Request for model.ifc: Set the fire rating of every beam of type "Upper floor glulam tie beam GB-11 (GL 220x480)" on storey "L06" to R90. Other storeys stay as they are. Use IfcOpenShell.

First a look at what the model holds.

```python
import ifcopenshell
import ifcopenshell.util.element

model = ifcopenshell.open("model.ifc")
print(model.schema)
storey = next(s for s in model.by_type("IfcBuildingStorey") if s.Name == "L06")
beams = [e for e in ifcopenshell.util.element.get_decomposition(storey) if e.is_a("IfcBeam")]
seen = {}
for e in beams:
    element_type = ifcopenshell.util.element.get_type(e)
    key = (element_type.Name if element_type != e and element_type else None, ifcopenshell.util.element.get_pset(e, "Pset_BeamCommon", "FireRating"))
    seen[key] = seen.get(key, 0) + 1
for (name, value), count in sorted(seen.items(), key=str):
    print(count, "x", name, "|", value)
```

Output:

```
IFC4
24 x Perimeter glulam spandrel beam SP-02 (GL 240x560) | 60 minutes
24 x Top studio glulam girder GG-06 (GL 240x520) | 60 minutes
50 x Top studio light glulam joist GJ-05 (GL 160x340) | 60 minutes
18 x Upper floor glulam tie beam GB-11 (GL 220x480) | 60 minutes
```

```python
import ifcopenshell
import ifcopenshell.api.pset
import ifcopenshell.util.element

model = ifcopenshell.open("model.ifc")

storey = next(s for s in model.by_type("IfcBuildingStorey") if s.Name == "L06")
beams = [e for e in ifcopenshell.util.element.get_decomposition(storey) if e.is_a("IfcBeam")]

count = 0
for e in beams:
    element_type = ifcopenshell.util.element.get_type(e)
    if element_type in (None, e) or element_type.Name != "Upper floor glulam tie beam GB-11 (GL 220x480)":
        continue
    # add_pset returns the element's existing set when there is one.
    pset = ifcopenshell.api.pset.add_pset(model, product=e, name="Pset_BeamCommon")
    ifcopenshell.api.pset.edit_pset(model, pset=pset, properties={"FireRating": "R90"})
    count += 1

print(count, "beams updated")

model.write("model-out.ifc")
```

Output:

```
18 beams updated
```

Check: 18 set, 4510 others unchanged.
